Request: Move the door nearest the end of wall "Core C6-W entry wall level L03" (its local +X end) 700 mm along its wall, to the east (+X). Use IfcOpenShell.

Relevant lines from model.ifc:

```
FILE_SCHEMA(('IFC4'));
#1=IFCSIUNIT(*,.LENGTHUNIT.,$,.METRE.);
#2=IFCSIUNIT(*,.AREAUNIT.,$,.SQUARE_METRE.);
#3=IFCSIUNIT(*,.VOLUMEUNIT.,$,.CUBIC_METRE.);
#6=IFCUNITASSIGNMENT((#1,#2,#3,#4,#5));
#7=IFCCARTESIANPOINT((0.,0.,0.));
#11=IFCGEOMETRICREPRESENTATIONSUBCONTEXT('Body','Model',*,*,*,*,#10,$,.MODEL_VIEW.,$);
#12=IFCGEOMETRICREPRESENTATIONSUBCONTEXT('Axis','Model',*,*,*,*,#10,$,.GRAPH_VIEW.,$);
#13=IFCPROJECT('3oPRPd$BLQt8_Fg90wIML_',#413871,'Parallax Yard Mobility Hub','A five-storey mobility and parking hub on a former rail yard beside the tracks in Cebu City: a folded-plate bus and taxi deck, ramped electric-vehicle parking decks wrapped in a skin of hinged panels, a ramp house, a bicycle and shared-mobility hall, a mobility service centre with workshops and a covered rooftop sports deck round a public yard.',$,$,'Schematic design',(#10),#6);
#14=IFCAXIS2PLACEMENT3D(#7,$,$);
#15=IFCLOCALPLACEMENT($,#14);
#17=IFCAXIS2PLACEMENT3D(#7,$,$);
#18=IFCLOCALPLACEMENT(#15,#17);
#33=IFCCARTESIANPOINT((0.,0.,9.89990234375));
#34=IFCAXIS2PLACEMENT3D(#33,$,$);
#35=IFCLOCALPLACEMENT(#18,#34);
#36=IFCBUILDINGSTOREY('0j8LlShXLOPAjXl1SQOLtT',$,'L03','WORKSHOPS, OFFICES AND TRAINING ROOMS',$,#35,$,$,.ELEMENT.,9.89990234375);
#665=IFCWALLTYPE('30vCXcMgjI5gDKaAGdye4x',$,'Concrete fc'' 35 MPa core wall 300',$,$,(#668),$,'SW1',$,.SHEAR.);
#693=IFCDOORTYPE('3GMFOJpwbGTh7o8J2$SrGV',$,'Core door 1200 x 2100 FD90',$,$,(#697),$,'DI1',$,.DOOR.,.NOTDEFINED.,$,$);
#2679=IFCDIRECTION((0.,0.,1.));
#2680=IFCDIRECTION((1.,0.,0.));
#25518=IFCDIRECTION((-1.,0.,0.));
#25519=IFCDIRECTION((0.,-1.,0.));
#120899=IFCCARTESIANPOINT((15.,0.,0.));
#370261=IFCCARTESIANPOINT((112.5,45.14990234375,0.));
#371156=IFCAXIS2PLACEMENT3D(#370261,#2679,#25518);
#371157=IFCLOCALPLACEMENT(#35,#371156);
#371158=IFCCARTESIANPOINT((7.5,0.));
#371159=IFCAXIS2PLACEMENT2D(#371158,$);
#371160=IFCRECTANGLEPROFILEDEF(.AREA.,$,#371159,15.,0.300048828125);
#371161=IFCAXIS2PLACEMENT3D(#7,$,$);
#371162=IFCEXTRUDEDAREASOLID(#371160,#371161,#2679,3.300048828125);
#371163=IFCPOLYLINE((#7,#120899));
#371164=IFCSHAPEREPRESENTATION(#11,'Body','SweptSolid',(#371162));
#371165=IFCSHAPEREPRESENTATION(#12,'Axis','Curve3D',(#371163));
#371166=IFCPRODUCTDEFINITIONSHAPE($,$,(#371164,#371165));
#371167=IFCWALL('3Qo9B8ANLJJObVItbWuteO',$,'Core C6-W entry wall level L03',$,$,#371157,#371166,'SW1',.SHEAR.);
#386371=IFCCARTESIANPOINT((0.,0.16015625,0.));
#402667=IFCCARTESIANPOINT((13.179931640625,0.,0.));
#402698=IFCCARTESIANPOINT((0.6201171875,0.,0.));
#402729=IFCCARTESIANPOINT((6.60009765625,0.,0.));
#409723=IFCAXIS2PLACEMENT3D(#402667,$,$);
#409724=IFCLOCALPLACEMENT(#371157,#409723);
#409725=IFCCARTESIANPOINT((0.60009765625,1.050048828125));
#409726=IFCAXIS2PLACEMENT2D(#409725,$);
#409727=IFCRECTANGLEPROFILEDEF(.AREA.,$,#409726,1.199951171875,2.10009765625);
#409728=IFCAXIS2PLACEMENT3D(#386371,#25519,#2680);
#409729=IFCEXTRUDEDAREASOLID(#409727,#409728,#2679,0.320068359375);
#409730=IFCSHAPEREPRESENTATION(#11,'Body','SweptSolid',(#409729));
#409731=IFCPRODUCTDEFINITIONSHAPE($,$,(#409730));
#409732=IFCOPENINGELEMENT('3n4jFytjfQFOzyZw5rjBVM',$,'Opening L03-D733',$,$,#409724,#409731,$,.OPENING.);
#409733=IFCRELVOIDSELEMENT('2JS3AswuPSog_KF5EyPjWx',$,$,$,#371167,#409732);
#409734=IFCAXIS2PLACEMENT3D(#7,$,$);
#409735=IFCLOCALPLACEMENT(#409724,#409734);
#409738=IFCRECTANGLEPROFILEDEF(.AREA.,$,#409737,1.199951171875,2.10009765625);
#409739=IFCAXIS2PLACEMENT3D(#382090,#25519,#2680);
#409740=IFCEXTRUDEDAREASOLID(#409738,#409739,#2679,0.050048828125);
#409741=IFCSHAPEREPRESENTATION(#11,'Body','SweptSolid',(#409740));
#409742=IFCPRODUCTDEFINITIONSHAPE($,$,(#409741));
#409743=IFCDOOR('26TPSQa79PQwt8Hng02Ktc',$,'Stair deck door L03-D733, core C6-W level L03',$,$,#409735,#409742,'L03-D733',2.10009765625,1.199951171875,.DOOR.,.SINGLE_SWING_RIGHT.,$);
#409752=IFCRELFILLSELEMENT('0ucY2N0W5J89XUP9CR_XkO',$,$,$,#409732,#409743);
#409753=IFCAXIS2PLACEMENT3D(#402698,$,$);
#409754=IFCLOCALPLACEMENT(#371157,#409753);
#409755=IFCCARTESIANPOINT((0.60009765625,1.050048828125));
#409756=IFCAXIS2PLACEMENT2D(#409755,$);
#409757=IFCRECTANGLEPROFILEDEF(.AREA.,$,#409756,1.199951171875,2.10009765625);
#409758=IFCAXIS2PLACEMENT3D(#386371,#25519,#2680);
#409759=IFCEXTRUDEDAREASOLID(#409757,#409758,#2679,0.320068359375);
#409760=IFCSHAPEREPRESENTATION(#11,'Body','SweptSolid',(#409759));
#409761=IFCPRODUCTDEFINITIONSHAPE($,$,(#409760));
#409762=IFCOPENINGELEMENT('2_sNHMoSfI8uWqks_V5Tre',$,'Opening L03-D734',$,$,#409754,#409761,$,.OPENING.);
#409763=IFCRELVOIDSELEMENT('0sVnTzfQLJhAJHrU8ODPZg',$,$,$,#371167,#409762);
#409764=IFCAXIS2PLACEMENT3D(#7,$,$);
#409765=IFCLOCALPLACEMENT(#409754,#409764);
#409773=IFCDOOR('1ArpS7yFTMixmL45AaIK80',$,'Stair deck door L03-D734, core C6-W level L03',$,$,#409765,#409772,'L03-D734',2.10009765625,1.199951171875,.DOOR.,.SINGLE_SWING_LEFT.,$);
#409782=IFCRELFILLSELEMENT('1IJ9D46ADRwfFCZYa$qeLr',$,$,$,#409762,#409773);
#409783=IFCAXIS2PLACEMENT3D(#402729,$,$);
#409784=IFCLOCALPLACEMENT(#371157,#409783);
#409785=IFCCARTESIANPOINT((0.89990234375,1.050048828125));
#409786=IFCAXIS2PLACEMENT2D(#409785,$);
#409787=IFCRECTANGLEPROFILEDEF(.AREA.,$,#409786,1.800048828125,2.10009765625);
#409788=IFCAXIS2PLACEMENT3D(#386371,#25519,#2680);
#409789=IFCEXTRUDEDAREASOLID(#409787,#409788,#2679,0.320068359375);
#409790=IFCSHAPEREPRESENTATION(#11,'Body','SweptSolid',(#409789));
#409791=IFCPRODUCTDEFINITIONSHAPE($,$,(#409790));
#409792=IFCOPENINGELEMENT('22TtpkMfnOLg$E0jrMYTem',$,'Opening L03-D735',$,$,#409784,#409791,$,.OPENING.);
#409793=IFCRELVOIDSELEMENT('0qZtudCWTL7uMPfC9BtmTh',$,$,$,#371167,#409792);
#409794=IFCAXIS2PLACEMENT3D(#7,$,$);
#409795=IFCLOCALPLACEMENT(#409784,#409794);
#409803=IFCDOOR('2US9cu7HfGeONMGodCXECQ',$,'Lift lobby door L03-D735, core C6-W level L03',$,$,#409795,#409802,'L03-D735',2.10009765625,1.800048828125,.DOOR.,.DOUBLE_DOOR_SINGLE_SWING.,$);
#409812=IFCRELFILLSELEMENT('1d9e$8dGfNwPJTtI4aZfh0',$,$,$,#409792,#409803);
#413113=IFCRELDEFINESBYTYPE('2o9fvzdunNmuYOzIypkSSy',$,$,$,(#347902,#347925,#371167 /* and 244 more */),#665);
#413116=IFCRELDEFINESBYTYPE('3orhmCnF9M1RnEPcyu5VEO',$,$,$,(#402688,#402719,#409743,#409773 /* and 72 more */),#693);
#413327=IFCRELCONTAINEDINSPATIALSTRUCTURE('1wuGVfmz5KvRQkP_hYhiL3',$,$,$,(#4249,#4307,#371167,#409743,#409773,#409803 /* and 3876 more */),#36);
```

```python
import ifcopenshell
import ifcopenshell.api.geometry
import ifcopenshell.util.placement
import ifcopenshell.util.unit

model = ifcopenshell.open("model.ifc")
unit_scale = ifcopenshell.util.unit.calculate_unit_scale(model)

door = model.by_guid("26TPSQa79PQwt8Hng02Ktc")
opening = door.FillsVoids[0].RelatingOpeningElement
wall = opening.VoidsElements[0].RelatingBuildingElement

wall_matrix = ifcopenshell.util.placement.get_local_placement(wall.ObjectPlacement)
shift = wall_matrix[:3, 0] * -0.7 / unit_scale
before = ifcopenshell.util.placement.get_local_placement(door.ObjectPlacement)[:3, 3].copy()

# The door is placed relative to its opening, so it follows when the opening moves.
matrix = ifcopenshell.util.placement.get_local_placement(opening.ObjectPlacement)
matrix[:3, 3] += shift
ifcopenshell.api.geometry.edit_object_placement(
    model, product=opening, matrix=matrix, is_si=False, should_transform_children=True
)

after = ifcopenshell.util.placement.get_local_placement(door.ObjectPlacement)[:3, 3]
print("door moved by", (after - before).round(3) + 0.0)

model.write("model_v2.ifc")
```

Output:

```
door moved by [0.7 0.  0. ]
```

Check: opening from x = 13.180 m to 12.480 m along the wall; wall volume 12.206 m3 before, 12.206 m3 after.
